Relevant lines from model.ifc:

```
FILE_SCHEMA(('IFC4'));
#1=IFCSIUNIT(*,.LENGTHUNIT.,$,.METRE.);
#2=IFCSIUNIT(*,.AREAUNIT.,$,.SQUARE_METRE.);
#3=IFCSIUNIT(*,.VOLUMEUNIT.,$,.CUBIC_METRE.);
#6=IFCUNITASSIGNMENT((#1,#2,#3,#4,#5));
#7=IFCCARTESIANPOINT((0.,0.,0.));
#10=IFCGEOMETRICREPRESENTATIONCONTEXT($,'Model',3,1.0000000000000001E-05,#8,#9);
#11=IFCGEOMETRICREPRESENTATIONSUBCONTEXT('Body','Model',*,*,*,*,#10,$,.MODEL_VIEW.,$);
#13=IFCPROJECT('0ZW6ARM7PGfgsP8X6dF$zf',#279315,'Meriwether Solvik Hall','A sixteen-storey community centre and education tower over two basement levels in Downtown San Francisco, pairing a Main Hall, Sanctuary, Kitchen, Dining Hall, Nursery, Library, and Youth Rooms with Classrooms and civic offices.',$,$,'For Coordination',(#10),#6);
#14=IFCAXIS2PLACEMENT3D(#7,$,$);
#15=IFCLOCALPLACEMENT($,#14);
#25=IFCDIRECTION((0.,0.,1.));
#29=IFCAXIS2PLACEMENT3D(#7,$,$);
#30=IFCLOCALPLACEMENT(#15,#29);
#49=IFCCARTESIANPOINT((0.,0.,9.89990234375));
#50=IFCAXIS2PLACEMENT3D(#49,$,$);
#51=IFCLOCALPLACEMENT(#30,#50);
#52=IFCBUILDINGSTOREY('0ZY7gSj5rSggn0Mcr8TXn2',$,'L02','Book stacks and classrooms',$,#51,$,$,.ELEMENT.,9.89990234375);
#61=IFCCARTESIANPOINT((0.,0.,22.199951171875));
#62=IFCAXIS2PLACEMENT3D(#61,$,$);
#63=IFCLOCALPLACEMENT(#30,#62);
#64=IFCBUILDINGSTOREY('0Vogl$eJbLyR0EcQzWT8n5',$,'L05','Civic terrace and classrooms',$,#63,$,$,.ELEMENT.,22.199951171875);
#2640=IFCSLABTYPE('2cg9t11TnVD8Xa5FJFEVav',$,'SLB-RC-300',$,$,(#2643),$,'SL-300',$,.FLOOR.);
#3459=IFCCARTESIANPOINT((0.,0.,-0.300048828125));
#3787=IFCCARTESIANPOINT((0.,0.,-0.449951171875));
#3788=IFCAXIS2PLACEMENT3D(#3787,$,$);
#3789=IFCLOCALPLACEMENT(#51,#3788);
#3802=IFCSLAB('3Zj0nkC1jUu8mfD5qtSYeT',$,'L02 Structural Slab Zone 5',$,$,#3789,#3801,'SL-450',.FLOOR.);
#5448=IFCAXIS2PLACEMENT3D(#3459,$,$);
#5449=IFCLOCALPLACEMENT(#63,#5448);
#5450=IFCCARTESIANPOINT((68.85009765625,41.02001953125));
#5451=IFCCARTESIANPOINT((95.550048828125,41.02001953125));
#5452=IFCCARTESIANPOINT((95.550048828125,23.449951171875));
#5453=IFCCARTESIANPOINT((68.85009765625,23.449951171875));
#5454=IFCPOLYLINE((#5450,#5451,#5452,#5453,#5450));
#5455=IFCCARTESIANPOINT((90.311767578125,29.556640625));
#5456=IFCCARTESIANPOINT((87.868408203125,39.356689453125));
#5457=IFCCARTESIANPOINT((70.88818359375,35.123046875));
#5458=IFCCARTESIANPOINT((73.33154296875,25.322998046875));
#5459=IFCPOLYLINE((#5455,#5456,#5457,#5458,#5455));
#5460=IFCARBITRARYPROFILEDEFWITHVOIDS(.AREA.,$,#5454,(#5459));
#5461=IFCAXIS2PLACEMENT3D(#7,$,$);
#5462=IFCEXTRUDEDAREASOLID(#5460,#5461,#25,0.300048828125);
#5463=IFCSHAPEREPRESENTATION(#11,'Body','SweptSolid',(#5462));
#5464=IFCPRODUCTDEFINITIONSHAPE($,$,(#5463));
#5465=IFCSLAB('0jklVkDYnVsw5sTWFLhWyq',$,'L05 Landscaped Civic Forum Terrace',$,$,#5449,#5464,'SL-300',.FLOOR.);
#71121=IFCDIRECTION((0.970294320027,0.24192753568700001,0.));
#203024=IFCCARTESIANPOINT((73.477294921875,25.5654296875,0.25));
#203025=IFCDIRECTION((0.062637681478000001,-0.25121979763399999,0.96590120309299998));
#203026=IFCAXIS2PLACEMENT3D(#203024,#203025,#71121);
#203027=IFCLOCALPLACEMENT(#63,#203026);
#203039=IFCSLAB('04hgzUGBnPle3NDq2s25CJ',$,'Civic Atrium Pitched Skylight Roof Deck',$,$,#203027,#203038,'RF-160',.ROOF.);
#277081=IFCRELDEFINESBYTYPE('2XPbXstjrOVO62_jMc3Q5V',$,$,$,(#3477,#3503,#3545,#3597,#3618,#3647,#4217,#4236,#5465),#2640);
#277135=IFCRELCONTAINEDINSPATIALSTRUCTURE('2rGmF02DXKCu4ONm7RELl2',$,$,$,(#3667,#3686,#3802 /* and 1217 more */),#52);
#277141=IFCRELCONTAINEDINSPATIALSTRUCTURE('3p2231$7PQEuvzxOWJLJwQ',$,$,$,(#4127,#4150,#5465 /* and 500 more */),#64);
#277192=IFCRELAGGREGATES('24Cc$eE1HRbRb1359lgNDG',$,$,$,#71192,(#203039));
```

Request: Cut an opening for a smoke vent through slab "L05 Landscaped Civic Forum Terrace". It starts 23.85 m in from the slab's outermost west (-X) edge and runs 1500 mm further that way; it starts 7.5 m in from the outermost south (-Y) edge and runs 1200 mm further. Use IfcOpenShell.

```python
import numpy as np
import ifcopenshell
import ifcopenshell.api.feature
import ifcopenshell.api.geometry
import ifcopenshell.api.root
import ifcopenshell.geom
import ifcopenshell.util.placement
import ifcopenshell.util.representation
import ifcopenshell.util.shape
import ifcopenshell.util.unit

model = ifcopenshell.open("model.ifc")
unit_scale = ifcopenshell.util.unit.calculate_unit_scale(model)
settings = ifcopenshell.geom.settings()


def volume(element):
    """Net volume in cubic metres, openings subtracted."""
    shape = ifcopenshell.geom.create_shape(settings, element)
    return ifcopenshell.util.shape.get_volume(shape.geometry)


slab = model.by_guid("0jklVkDYnVsw5sTWFLhWyq")
before = volume(slab)

# Extent in the slab's own axes, in metres. The edges named are its -X and -Y sides.
slab_shape = ifcopenshell.geom.create_shape(settings, slab)
vertices = ifcopenshell.util.shape.get_vertices(slab_shape.geometry)
x_min, y_min, bottom = vertices.min(axis=0)
top = vertices[:, 2].max()

opening = ifcopenshell.api.root.create_entity(model, ifc_class="IfcOpeningElement", name="Smoke vent opening", predefined_type="OPENING")
context = ifcopenshell.util.representation.get_context(model, "Model", "Body", "MODEL_VIEW")
width, depth = 1.5, 1.2
outline = [(0.0, 0.0), (width, 0.0), (width, depth), (0.0, depth), (0.0, 0.0)]
# Overshoot both faces by 50 mm so the cut is clean.
shape = ifcopenshell.api.geometry.add_slab_representation(
    model, context=context, depth=top - bottom + 0.1, polyline=outline
)
ifcopenshell.api.geometry.assign_representation(model, product=opening, representation=shape)

matrix = ifcopenshell.util.placement.get_local_placement(slab.ObjectPlacement)
matrix[:, 3] = matrix @ np.append(np.array([x_min + 23.85, y_min + 7.5, bottom - 0.05]) / unit_scale, 1.0)
ifcopenshell.api.geometry.edit_object_placement(model, product=opening, matrix=matrix, is_si=False)
ifcopenshell.api.feature.add_feature(model, feature=opening, element=slab)

after = volume(slab)

print(f"slab volume {before:.3f} -> {after:.3f} m3")

model.write("model_v2.ifc")
```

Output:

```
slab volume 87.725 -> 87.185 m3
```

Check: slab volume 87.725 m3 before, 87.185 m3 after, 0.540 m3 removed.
